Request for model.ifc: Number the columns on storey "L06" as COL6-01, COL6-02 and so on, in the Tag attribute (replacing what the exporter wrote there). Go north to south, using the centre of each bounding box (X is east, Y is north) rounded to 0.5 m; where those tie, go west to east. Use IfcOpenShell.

First a look at what the model holds.

```python
import ifcopenshell
import ifcopenshell.util.element
import ifcopenshell.util.placement

model = ifcopenshell.open("model.ifc")
print(model.schema)
storey = next(s for s in model.by_type("IfcBuildingStorey") if s.Name == "L06")
columns = [e for e in ifcopenshell.util.element.get_decomposition(storey) if e.is_a("IfcColumn")]
for e in sorted(columns, key=lambda e: e.id()):
    origin = ifcopenshell.util.placement.get_local_placement(e.ObjectPlacement)[:3, 3]
    print(e.id(), e.Tag, e.Name, origin.round(2) + 0.0, sep=" | ")
```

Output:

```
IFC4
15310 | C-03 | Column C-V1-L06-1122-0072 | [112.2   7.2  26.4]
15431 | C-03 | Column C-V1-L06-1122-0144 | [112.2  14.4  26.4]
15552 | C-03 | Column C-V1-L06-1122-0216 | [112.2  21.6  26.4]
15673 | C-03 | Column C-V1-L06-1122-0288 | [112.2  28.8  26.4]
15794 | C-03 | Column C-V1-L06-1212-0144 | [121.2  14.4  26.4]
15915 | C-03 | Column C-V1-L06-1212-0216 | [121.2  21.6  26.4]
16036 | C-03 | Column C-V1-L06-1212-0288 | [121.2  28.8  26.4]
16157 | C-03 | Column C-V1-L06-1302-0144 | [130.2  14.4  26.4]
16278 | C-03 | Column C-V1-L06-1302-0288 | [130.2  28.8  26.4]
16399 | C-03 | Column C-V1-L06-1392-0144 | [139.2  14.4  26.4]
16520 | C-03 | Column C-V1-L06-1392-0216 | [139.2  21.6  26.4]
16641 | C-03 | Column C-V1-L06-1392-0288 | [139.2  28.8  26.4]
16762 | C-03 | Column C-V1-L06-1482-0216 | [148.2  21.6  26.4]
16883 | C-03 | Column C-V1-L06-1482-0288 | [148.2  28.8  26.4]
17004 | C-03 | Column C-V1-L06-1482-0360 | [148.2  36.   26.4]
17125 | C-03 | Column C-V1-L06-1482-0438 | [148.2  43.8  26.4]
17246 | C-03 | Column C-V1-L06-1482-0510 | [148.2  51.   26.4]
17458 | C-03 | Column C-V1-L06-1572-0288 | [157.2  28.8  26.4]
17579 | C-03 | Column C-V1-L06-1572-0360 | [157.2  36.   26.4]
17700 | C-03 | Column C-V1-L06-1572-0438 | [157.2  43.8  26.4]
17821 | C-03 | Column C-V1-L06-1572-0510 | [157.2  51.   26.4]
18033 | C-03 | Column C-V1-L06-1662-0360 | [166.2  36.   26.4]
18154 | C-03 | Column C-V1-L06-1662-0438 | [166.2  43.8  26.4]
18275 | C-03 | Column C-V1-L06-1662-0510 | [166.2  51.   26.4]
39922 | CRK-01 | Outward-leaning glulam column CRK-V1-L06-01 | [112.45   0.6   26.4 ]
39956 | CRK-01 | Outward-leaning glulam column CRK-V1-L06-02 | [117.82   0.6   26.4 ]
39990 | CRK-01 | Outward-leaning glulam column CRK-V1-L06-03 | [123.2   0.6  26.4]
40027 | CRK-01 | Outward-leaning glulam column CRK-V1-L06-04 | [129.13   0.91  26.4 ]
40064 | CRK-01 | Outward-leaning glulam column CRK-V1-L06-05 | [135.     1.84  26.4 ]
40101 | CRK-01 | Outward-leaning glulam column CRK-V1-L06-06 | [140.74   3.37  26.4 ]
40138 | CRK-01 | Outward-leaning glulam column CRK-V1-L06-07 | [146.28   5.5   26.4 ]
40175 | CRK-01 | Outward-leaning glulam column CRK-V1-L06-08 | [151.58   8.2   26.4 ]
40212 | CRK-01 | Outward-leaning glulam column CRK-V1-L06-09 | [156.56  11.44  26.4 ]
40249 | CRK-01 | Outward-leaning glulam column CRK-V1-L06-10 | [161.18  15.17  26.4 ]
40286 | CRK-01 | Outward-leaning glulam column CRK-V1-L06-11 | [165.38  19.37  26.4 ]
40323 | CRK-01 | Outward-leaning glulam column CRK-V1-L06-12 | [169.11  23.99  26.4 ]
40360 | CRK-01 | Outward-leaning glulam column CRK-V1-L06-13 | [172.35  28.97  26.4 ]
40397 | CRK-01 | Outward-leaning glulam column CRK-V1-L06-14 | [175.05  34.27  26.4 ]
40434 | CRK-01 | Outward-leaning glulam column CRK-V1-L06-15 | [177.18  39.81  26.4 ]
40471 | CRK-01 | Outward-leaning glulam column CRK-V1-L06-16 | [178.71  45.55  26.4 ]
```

```python
import ifcopenshell
import ifcopenshell.geom
import ifcopenshell.util.element
import ifcopenshell.util.shape

model = ifcopenshell.open("model.ifc")
settings = ifcopenshell.geom.settings()
settings.set("use-world-coords", True)


def centre(element):
    shape = ifcopenshell.geom.create_shape(settings, element)
    return ifcopenshell.util.shape.get_bbox_centroid(shape.geometry)


storey = next(s for s in model.by_type("IfcBuildingStorey") if s.Name == "L06")
columns = [e for e in ifcopenshell.util.element.get_decomposition(storey) if e.is_a("IfcColumn")]

# Insertion points can sit at a corner or the storey origin, so sort by the geometry (in metres).
centres = {e: centre(e) for e in columns}
columns.sort(key=lambda e: (-round(centres[e][1] / 0.5), centres[e][0]))

for i, e in enumerate(columns, start=1):
    number = f"COL6-{i:02d}"
    e.Tag = number
    print(e.id(), number)

model.write("model_v2.ifc")
```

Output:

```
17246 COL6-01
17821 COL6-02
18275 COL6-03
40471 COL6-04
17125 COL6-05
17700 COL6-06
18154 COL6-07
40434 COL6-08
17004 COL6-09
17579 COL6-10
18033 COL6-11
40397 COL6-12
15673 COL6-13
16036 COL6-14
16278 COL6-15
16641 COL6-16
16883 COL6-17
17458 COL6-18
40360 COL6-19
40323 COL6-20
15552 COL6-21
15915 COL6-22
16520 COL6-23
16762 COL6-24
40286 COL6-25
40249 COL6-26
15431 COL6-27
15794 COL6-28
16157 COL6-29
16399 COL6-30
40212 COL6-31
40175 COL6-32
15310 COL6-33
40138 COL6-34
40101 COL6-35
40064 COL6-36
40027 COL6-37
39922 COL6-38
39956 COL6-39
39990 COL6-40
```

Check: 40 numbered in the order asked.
